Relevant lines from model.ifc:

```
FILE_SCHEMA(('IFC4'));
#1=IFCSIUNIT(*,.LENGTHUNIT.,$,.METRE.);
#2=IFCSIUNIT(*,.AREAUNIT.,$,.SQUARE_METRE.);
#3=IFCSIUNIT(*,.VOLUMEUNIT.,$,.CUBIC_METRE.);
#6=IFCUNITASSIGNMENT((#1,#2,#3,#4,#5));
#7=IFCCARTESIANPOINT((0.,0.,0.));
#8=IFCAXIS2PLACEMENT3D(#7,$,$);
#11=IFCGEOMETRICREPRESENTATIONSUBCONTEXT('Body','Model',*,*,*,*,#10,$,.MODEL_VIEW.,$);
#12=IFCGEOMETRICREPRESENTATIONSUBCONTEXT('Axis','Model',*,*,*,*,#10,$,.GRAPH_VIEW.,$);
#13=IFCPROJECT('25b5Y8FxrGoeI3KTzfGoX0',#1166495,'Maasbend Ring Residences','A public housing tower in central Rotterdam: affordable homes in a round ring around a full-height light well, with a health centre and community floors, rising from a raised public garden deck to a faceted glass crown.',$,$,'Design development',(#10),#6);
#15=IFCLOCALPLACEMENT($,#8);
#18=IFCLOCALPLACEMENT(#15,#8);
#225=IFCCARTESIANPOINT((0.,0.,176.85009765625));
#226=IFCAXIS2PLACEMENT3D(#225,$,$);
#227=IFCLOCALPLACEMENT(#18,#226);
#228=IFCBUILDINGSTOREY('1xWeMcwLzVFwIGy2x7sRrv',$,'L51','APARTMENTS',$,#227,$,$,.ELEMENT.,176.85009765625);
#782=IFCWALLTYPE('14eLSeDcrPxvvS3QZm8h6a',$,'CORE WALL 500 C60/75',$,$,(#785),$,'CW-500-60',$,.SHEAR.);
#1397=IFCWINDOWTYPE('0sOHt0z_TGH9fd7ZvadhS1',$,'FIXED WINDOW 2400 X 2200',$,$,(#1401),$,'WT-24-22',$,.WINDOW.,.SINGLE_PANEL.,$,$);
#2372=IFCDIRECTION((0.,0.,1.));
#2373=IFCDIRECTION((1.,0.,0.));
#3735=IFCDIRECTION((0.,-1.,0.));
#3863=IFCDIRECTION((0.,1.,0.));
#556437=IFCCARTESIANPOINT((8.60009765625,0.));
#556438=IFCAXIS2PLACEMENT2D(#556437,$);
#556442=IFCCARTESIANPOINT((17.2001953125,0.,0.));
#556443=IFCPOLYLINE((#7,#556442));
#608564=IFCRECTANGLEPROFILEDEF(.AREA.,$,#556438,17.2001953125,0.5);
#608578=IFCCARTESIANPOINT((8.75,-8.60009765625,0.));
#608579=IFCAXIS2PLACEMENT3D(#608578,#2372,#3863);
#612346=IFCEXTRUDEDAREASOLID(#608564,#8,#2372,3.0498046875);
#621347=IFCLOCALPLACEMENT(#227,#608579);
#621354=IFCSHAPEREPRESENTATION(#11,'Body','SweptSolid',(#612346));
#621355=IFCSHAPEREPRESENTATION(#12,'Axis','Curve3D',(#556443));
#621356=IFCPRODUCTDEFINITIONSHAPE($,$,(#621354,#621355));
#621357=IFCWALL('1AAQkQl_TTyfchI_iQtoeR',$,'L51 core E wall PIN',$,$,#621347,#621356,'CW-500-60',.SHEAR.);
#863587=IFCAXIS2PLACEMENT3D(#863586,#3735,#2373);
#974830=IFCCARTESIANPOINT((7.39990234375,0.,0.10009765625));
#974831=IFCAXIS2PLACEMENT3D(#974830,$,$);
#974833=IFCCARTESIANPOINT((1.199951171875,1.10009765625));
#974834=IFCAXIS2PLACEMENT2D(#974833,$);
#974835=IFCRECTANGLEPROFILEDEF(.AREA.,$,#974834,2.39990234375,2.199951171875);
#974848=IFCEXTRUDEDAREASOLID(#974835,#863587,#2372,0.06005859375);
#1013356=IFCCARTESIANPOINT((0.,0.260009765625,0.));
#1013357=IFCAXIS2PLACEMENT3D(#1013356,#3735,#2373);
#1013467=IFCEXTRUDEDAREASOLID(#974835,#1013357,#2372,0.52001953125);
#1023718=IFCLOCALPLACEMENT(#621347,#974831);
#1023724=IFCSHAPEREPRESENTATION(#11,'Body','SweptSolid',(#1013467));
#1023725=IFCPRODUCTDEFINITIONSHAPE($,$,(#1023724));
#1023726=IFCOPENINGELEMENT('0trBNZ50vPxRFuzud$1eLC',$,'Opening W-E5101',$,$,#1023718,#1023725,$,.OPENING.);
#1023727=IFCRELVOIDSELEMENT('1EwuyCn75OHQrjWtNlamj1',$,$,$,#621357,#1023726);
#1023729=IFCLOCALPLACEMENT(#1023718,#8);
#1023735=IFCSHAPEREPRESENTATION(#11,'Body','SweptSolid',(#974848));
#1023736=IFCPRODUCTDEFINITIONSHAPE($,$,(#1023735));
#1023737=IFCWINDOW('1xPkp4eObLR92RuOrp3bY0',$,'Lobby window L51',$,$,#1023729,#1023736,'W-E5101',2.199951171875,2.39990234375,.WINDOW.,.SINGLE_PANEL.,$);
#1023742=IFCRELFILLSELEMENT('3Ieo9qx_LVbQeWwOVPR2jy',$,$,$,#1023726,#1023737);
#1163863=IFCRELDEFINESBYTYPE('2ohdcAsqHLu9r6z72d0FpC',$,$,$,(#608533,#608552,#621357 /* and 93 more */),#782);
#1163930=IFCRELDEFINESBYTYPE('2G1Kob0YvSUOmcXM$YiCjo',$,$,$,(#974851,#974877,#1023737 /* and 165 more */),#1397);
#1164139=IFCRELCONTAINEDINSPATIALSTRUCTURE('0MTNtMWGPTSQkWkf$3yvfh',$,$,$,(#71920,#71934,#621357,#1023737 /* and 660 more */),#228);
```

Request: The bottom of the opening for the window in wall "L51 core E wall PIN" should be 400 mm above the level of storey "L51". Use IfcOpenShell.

```python
import numpy as np
import ifcopenshell
import ifcopenshell.api.geometry
import ifcopenshell.geom
import ifcopenshell.util.element
import ifcopenshell.util.placement
import ifcopenshell.util.shape
import ifcopenshell.util.unit

model = ifcopenshell.open("model.ifc")
unit_scale = ifcopenshell.util.unit.calculate_unit_scale(model)

window = model.by_guid("1xPkp4eObLR92RuOrp3bY0")
opening = window.FillsVoids[0].RelatingOpeningElement
storey = ifcopenshell.util.element.get_container(window, ifc_class="IfcBuildingStorey")
level = ifcopenshell.util.placement.get_local_placement(storey.ObjectPlacement)[2, 3]

# The opening's origin need not be at the sill, so measure its lowest point.
shape = ifcopenshell.geom.create_shape(ifcopenshell.geom.settings(), opening)
bottom = ifcopenshell.util.shape.get_shape_bottom_elevation(shape, shape.geometry) / unit_scale
dz = level + 0.4 / unit_scale - bottom

shift = np.array([0.0, 0.0, dz])
# The window is placed relative to its opening, so it follows when the opening moves.
matrix = ifcopenshell.util.placement.get_local_placement(opening.ObjectPlacement)
matrix[:3, 3] += shift
ifcopenshell.api.geometry.edit_object_placement(
    model, product=opening, matrix=matrix, is_si=False, should_transform_children=True
)

print(f"moved by {dz * unit_scale:+.3f} m")

model.write("model_v2.ifc")
```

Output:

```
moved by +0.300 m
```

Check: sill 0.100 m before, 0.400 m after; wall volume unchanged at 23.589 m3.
